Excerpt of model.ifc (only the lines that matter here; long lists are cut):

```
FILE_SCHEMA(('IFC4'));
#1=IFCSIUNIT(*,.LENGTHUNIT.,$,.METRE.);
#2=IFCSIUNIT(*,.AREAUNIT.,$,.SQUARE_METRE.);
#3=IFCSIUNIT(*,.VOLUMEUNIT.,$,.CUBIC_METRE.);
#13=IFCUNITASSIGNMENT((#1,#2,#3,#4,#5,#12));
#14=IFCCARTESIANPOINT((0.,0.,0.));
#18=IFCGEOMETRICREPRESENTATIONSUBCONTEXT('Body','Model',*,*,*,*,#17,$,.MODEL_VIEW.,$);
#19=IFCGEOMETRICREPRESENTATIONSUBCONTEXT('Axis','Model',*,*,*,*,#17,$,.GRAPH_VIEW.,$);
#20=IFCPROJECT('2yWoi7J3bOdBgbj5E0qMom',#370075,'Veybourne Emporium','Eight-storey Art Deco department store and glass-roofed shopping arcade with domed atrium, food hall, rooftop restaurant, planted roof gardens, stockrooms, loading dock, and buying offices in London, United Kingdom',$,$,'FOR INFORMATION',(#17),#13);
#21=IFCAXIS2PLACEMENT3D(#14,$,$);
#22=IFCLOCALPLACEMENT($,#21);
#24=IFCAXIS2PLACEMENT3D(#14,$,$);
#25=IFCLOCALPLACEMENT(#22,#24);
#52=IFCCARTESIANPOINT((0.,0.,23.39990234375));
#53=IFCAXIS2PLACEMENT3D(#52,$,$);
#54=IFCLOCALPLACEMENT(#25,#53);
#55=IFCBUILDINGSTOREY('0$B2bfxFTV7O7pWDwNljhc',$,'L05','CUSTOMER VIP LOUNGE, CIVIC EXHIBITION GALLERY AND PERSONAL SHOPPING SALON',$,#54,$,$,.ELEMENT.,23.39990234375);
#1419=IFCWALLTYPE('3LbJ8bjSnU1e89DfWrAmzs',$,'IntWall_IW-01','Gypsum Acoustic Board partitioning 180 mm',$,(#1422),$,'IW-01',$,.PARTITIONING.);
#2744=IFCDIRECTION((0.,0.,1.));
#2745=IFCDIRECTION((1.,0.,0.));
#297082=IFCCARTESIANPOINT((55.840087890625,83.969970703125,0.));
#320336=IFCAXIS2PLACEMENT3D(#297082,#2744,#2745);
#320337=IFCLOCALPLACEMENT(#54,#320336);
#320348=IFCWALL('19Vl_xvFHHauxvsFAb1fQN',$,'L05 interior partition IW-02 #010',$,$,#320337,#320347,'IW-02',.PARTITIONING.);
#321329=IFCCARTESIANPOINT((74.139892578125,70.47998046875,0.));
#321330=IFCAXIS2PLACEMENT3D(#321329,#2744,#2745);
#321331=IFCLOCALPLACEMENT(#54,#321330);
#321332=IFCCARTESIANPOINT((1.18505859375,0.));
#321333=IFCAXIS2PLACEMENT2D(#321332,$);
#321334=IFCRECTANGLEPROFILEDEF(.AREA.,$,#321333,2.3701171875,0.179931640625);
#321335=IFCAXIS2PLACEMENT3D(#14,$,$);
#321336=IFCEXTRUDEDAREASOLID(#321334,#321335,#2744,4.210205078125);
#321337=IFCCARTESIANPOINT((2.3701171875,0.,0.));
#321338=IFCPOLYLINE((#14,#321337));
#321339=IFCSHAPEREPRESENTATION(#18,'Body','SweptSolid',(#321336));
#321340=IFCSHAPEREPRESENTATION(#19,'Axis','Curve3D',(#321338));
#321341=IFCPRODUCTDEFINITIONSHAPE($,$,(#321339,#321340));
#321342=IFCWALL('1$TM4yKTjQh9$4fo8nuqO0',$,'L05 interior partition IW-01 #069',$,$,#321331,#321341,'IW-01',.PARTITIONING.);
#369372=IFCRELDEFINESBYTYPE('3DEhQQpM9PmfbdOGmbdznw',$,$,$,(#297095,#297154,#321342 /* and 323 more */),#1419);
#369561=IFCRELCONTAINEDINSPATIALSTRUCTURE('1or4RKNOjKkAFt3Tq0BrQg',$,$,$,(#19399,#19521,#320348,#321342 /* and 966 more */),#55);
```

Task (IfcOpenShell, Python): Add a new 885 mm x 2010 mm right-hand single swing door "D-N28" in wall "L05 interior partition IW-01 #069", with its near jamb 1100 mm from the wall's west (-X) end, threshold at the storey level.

```python
import numpy as np
import ifcopenshell
import ifcopenshell.api.feature
import ifcopenshell.api.geometry
import ifcopenshell.api.root
import ifcopenshell.api.spatial
import ifcopenshell.geom
import ifcopenshell.util.element
import ifcopenshell.util.placement
import ifcopenshell.util.representation
import ifcopenshell.util.shape
import ifcopenshell.util.unit

model = ifcopenshell.open("model.ifc")
unit_scale = ifcopenshell.util.unit.calculate_unit_scale(model)
settings = ifcopenshell.geom.settings()


def volume(element):
    """Net volume in cubic metres, openings subtracted."""
    shape = ifcopenshell.geom.create_shape(settings, element)
    return ifcopenshell.util.shape.get_volume(shape.geometry)


wall = model.by_guid("1$TM4yKTjQh9$4fo8nuqO0")
storey = ifcopenshell.util.element.get_container(wall, ifc_class="IfcBuildingStorey")
context = ifcopenshell.util.representation.get_context(model, "Model", "Body", "MODEL_VIEW")
before = volume(wall)

width, height, from_end, sill = 0.885, 2.01, 1.1, 0.0  # metres

# The wall runs along its own X axis, and the end named is its -X end.
wall_shape = ifcopenshell.geom.create_shape(settings, wall)
x, y, z = ifcopenshell.util.shape.get_vertices(wall_shape.geometry).T
start = x.min() + from_end
face, thickness = float(y.min()), float(y.max() - y.min())
wall_matrix = ifcopenshell.util.placement.get_local_placement(wall.ObjectPlacement)
level = ifcopenshell.util.placement.get_local_placement(storey.ObjectPlacement)[2, 3]


def in_wall(x, y):
    """Placement at x, y metres in the wall's axes, at sill height."""
    matrix = wall_matrix.copy()
    matrix[:, 3] = wall_matrix @ np.array([x / unit_scale, y / unit_scale, 0.0, 1.0])
    matrix[2, 3] = level + sill / unit_scale
    return matrix


# Opening: a box that overshoots both wall faces by 50 mm.
opening = ifcopenshell.api.root.create_entity(model, ifc_class="IfcOpeningElement", predefined_type="OPENING")
box = ifcopenshell.api.geometry.add_wall_representation(
    model, context=context, length=width, height=height, thickness=thickness + 0.1
)
ifcopenshell.api.geometry.assign_representation(model, product=opening, representation=box)
ifcopenshell.api.geometry.edit_object_placement(model, product=opening, matrix=in_wall(start, face - 0.05), is_si=False)
ifcopenshell.api.feature.add_feature(model, feature=opening, element=wall)

door = ifcopenshell.api.root.create_entity(model, ifc_class="IfcDoor", name="D-N28", predefined_type="DOOR")
door.OverallWidth, door.OverallHeight = width / unit_scale, height / unit_scale
door.OperationType = "SINGLE_SWING_RIGHT"
body = ifcopenshell.api.geometry.add_door_representation(
    model,
    context=context,
    overall_width=door.OverallWidth,
    overall_height=door.OverallHeight,
    operation_type="SINGLE_SWING_RIGHT",
    lining_properties={"LiningDepth": thickness / unit_scale, "ThresholdDepth": thickness / unit_scale},
)
ifcopenshell.api.geometry.assign_representation(model, product=door, representation=body)
ifcopenshell.api.spatial.assign_container(model, products=[door], relating_structure=storey)
ifcopenshell.api.feature.add_filling(model, opening=opening, element=door)

# The lining spans the wall, so the door starts at the wall face.
ifcopenshell.api.geometry.edit_object_placement(model, product=door, matrix=in_wall(start, face), is_si=False)

after = volume(wall)

print(f"wall volume {before:.3f} -> {after:.3f} m3")

model.write("model_updated.ifc")
```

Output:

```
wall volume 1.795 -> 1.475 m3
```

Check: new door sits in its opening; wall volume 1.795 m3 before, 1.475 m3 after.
